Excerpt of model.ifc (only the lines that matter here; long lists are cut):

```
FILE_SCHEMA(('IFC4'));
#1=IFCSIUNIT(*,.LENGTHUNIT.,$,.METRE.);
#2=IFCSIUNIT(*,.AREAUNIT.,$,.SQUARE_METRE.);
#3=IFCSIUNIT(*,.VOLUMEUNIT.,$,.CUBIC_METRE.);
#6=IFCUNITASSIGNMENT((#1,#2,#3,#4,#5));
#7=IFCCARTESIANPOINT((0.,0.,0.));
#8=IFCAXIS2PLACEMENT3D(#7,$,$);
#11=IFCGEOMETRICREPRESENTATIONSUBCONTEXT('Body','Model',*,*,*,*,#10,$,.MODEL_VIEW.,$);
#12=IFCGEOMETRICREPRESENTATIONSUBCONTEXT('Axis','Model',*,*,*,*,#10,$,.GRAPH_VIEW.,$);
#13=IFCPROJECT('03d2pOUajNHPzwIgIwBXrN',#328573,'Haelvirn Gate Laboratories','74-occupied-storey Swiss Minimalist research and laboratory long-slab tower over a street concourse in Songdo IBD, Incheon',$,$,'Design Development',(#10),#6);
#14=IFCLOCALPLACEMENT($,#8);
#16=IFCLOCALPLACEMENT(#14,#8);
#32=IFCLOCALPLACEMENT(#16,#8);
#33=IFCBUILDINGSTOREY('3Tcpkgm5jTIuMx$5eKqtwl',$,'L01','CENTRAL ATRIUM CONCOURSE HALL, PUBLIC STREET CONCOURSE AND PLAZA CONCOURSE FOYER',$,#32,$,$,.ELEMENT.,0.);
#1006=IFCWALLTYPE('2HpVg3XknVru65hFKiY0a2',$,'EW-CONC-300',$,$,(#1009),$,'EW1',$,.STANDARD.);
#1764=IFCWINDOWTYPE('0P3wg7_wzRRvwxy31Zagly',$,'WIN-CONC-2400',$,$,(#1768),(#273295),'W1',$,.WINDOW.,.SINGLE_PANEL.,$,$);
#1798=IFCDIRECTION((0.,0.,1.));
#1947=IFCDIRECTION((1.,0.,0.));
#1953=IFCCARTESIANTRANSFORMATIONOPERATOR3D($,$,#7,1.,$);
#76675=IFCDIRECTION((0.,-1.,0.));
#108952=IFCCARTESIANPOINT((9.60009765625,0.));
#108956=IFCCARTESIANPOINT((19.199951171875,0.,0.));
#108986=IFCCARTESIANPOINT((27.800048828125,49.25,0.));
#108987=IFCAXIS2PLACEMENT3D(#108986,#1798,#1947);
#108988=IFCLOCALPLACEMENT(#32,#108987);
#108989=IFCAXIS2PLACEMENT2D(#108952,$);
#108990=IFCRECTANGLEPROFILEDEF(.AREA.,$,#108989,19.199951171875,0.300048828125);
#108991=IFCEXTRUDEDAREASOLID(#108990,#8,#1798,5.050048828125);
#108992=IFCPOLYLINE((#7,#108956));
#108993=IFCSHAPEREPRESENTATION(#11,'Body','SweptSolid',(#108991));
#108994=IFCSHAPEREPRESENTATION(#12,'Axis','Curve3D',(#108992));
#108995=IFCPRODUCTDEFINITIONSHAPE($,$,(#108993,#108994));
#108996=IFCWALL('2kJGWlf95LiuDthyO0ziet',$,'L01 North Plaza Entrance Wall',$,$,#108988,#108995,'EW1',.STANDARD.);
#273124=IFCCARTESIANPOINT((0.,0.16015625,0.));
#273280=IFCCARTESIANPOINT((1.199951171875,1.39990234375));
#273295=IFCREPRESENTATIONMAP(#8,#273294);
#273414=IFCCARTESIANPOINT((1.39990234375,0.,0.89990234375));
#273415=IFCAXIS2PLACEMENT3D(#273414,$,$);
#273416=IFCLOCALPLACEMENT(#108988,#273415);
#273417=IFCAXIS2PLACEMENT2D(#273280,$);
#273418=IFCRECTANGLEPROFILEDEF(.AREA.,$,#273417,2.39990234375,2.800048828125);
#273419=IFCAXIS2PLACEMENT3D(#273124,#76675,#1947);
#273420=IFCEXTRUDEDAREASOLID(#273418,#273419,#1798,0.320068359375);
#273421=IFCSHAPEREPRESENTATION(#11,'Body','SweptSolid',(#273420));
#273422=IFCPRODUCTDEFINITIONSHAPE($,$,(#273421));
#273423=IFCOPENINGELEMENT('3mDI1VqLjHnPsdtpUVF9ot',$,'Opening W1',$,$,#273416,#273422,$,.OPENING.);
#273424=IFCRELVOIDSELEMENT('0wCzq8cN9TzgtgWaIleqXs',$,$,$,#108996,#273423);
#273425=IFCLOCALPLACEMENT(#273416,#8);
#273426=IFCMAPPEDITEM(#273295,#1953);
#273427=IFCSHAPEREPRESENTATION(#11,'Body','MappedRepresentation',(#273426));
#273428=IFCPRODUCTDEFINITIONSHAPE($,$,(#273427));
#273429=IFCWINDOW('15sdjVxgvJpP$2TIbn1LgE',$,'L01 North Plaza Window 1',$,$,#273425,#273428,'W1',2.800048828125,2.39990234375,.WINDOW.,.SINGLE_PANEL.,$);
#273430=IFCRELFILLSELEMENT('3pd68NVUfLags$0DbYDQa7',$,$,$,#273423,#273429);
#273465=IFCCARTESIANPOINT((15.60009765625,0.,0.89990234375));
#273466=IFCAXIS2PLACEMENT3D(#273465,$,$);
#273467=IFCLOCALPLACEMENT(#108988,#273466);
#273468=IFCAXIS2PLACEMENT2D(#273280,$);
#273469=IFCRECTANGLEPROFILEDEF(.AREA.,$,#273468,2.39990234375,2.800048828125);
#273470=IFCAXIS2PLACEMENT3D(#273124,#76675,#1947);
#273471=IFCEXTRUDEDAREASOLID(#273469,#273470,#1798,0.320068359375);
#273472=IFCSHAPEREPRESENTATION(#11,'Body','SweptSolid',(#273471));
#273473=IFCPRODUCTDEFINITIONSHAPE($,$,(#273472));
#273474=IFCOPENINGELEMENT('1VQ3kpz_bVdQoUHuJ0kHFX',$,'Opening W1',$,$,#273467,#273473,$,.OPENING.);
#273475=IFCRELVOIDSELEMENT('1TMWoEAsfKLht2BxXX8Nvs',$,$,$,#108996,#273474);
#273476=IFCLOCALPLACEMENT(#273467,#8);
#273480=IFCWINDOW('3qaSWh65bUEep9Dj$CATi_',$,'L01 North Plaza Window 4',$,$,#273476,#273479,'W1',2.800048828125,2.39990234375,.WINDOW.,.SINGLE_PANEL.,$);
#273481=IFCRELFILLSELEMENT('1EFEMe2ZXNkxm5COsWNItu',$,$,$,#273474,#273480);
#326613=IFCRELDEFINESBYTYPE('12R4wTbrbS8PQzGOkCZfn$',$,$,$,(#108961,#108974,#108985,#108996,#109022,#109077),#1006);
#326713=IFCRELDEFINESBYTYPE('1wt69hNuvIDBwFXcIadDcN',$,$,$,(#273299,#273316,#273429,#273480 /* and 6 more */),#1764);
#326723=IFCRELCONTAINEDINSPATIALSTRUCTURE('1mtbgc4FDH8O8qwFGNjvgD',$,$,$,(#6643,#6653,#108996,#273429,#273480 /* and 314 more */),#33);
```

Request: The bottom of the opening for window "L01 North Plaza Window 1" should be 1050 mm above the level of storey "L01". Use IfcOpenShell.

```python
import numpy as np
import ifcopenshell
import ifcopenshell.api.geometry
import ifcopenshell.geom
import ifcopenshell.util.element
import ifcopenshell.util.placement
import ifcopenshell.util.shape
import ifcopenshell.util.unit

model = ifcopenshell.open("model.ifc")
unit_scale = ifcopenshell.util.unit.calculate_unit_scale(model)

window = model.by_guid("15sdjVxgvJpP$2TIbn1LgE")
opening = window.FillsVoids[0].RelatingOpeningElement
storey = ifcopenshell.util.element.get_container(window, ifc_class="IfcBuildingStorey")
level = ifcopenshell.util.placement.get_local_placement(storey.ObjectPlacement)[2, 3]

# The opening's origin need not be at the sill, so measure its lowest point.
shape = ifcopenshell.geom.create_shape(ifcopenshell.geom.settings(), opening)
bottom = ifcopenshell.util.shape.get_shape_bottom_elevation(shape, shape.geometry) / unit_scale
dz = level + 1.05 - bottom

shift = np.array([0.0, 0.0, dz])
# The window is placed relative to its opening, so it follows when the opening moves.
matrix = ifcopenshell.util.placement.get_local_placement(opening.ObjectPlacement)
matrix[:3, 3] += shift
ifcopenshell.api.geometry.edit_object_placement(
    model, product=opening, matrix=matrix, is_si=False, should_transform_children=True
)

print(f"moved by {dz * unit_scale:+.3f} m")

model.write("model_v2.ifc")
```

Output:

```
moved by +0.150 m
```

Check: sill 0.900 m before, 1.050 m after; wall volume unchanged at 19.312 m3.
